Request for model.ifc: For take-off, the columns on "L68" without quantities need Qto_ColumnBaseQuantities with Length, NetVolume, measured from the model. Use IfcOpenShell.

First a look at what the model holds.

```python
import ifcopenshell
import ifcopenshell.util.element
import ifcopenshell.util.unit

model = ifcopenshell.open("model.ifc")
print(model.schema)
for unit_type in ("LENGTHUNIT", "AREAUNIT", "VOLUMEUNIT"):
    print(unit_type, ifcopenshell.util.unit.calculate_unit_scale(model, unit_type))
storey = next(s for s in model.by_type("IfcBuildingStorey") if s.Name == "L68")
columns = [e for e in ifcopenshell.util.element.get_decomposition(storey) if e.is_a("IfcColumn")]
for e in sorted(columns, key=lambda e: e.id()):
    print(e.id(), e.is_a(), e.Name, list(ifcopenshell.util.element.get_psets(e, qtos_only=True)), sep=" | ")
```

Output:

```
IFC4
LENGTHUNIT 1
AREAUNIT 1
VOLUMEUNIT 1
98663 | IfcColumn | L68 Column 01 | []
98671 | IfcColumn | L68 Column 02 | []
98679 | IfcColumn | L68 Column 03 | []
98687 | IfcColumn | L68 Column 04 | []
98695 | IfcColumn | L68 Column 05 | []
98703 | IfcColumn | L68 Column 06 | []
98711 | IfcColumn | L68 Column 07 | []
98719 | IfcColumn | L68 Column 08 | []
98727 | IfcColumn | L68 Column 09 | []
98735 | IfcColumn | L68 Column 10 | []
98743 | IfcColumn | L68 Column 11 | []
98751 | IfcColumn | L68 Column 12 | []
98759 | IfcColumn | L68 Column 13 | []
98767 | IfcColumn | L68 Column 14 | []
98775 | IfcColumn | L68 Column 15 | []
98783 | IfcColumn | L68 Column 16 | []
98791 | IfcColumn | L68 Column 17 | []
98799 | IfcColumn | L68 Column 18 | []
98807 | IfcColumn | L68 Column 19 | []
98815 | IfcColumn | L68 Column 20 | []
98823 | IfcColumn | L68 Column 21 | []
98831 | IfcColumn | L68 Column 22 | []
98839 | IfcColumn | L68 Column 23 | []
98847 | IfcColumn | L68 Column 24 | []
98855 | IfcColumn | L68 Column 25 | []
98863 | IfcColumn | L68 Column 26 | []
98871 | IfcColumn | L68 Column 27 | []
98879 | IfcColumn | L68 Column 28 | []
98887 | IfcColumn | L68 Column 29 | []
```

```python
import ifcopenshell
import ifcopenshell.api.pset
import ifcopenshell.geom
import ifcopenshell.util.element
import ifcopenshell.util.shape
import ifcopenshell.util.unit

model = ifcopenshell.open("model.ifc")
unit_scale = ifcopenshell.util.unit.calculate_unit_scale(model)
volume_scale = ifcopenshell.util.unit.calculate_unit_scale(model, "VOLUMEUNIT")
settings = ifcopenshell.geom.settings()

storey = next(s for s in model.by_type("IfcBuildingStorey") if s.Name == "L68")
columns = [e for e in ifcopenshell.util.element.get_decomposition(storey) if e.is_a("IfcColumn")]

for e in sorted(columns, key=lambda e: e.id()):
    if ifcopenshell.util.element.get_psets(e, qtos_only=True, should_inherit=False):
        continue
    # Geometry comes back in metres, in the element's own axes.
    shape = ifcopenshell.geom.create_shape(settings, e)
    values = {
        "Length": ifcopenshell.util.shape.get_z(shape.geometry) / unit_scale,
        "NetVolume": ifcopenshell.util.shape.get_volume(shape.geometry) / volume_scale,
    }
    qto = ifcopenshell.api.pset.add_qto(model, product=e, name="Qto_ColumnBaseQuantities")
    ifcopenshell.api.pset.edit_qto(model, qto=qto, properties=values)
    print(e.id(), {k: round(v, 3) for k, v in values.items()})

model.write("model_updated.ifc")
```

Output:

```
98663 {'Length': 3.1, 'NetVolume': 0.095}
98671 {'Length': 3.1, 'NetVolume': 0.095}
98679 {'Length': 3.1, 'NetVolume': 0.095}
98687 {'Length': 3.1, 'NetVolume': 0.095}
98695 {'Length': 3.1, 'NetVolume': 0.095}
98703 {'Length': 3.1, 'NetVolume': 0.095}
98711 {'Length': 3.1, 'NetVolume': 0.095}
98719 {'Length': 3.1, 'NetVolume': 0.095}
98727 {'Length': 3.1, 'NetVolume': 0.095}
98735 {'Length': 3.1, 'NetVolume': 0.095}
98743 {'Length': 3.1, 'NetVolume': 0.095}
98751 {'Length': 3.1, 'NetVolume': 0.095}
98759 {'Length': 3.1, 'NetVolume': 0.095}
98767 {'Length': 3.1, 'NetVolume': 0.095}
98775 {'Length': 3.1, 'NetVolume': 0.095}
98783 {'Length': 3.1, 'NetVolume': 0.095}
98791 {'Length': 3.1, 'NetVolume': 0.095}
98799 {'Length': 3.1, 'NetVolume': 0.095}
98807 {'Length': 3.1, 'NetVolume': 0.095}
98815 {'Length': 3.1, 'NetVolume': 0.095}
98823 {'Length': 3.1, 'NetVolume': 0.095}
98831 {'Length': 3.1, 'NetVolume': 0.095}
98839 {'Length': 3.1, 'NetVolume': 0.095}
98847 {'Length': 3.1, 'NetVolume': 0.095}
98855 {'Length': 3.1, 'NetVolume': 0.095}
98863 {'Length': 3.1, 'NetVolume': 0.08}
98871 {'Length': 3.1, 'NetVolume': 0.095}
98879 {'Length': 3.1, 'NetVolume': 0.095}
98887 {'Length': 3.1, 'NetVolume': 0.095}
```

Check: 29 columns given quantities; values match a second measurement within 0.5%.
